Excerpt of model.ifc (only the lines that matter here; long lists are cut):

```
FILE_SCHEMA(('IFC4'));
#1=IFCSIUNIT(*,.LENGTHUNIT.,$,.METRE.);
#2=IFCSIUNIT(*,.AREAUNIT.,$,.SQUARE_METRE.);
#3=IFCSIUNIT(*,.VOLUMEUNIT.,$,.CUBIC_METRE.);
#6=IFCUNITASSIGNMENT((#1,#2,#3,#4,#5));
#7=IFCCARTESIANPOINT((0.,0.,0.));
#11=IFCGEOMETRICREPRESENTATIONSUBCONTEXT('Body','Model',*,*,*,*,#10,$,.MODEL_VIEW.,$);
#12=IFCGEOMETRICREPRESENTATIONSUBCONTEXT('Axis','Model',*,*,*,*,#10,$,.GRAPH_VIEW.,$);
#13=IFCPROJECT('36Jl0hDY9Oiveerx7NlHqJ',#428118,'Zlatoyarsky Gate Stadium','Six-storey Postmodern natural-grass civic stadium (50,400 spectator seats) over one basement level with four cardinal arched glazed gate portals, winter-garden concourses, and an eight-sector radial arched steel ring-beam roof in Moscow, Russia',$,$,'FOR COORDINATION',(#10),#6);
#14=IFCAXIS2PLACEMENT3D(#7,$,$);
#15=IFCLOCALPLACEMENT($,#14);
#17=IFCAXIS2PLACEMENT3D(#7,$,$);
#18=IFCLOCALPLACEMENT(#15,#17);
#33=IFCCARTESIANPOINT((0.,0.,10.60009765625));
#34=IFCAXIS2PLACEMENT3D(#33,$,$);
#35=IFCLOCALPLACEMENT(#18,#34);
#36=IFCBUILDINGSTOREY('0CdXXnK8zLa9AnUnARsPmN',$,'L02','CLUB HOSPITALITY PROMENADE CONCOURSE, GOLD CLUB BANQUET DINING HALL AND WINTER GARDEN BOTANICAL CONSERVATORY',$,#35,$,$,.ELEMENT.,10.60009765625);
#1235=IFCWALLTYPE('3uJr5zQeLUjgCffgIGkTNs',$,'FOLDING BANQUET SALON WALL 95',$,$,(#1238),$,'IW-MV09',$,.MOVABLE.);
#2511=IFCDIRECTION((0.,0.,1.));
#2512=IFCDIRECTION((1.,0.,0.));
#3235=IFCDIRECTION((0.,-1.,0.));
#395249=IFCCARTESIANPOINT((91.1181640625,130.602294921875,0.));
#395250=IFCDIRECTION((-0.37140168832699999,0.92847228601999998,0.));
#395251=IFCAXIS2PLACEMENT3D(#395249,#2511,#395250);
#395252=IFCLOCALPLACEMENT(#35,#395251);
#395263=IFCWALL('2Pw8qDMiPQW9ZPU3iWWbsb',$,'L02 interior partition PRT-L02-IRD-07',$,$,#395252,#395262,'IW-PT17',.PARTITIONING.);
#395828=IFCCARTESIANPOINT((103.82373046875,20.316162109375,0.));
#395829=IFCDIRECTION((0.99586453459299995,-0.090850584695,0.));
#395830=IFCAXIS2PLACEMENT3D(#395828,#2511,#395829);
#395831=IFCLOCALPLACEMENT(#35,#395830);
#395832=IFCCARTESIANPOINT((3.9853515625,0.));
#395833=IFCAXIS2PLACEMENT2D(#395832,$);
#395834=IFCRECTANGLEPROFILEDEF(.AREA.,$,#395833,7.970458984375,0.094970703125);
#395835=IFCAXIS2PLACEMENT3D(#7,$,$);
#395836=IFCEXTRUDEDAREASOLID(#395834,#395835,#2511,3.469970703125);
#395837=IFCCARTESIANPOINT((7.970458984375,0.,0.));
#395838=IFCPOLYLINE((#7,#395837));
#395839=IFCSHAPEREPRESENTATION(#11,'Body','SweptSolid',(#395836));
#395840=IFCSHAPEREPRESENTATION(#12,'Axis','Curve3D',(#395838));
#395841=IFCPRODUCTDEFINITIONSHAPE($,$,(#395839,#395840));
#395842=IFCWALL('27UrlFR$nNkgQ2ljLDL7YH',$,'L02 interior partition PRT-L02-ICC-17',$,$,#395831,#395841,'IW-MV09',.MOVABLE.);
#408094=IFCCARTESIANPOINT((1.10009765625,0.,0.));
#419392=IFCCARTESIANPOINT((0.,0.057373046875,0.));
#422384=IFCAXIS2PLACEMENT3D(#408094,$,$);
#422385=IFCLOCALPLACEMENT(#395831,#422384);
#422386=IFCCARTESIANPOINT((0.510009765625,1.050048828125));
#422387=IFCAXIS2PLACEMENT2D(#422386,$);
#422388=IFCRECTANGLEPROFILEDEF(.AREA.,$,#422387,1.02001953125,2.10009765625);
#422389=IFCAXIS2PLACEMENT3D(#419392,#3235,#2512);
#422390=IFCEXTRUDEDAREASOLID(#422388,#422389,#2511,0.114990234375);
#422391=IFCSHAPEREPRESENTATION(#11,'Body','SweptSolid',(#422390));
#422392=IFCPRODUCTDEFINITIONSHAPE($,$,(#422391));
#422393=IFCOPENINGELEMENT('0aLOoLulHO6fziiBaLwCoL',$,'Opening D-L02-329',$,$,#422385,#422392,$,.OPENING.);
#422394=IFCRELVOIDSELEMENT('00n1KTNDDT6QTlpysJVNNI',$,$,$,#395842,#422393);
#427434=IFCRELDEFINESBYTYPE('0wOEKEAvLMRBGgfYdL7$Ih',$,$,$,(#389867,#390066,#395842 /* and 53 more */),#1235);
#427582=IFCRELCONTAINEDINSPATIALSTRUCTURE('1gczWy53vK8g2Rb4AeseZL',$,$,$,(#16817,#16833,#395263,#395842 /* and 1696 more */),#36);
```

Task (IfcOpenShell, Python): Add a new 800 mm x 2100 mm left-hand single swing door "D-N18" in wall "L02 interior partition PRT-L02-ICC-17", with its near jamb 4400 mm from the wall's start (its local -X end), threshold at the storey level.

```python
import numpy as np
import ifcopenshell
import ifcopenshell.api.feature
import ifcopenshell.api.geometry
import ifcopenshell.api.root
import ifcopenshell.api.spatial
import ifcopenshell.geom
import ifcopenshell.util.element
import ifcopenshell.util.placement
import ifcopenshell.util.representation
import ifcopenshell.util.shape
import ifcopenshell.util.unit

model = ifcopenshell.open("model.ifc")
unit_scale = ifcopenshell.util.unit.calculate_unit_scale(model)
settings = ifcopenshell.geom.settings()


def volume(element):
    """Net volume in cubic metres, openings subtracted."""
    shape = ifcopenshell.geom.create_shape(settings, element)
    return ifcopenshell.util.shape.get_volume(shape.geometry)


wall = model.by_id(395842)
storey = ifcopenshell.util.element.get_container(wall, ifc_class="IfcBuildingStorey")
context = ifcopenshell.util.representation.get_context(model, "Model", "Body", "MODEL_VIEW")
before = volume(wall)

width, height, from_end, sill = 0.8, 2.1, 4.4, 0.0  # metres

# The wall runs along its own X axis, and the end named is its -X end.
wall_shape = ifcopenshell.geom.create_shape(settings, wall)
x, y, z = ifcopenshell.util.shape.get_vertices(wall_shape.geometry).T
start = x.min() + from_end
face, thickness = float(y.min()), float(y.max() - y.min())
wall_matrix = ifcopenshell.util.placement.get_local_placement(wall.ObjectPlacement)
level = ifcopenshell.util.placement.get_local_placement(storey.ObjectPlacement)[2, 3]


def in_wall(x, y):
    """Placement at x, y metres in the wall's axes, at sill height."""
    matrix = wall_matrix.copy()
    matrix[:, 3] = wall_matrix @ np.array([x / unit_scale, y / unit_scale, 0.0, 1.0])
    matrix[2, 3] = level + sill / unit_scale
    return matrix


# Opening: a box that overshoots both wall faces by 50 mm.
opening = ifcopenshell.api.root.create_entity(model, ifc_class="IfcOpeningElement", predefined_type="OPENING")
box = ifcopenshell.api.geometry.add_wall_representation(
    model, context=context, length=width, height=height, thickness=thickness + 0.1
)
ifcopenshell.api.geometry.assign_representation(model, product=opening, representation=box)
ifcopenshell.api.geometry.edit_object_placement(model, product=opening, matrix=in_wall(start, face - 0.05), is_si=False)
ifcopenshell.api.feature.add_feature(model, feature=opening, element=wall)

door = ifcopenshell.api.root.create_entity(model, ifc_class="IfcDoor", name="D-N18", predefined_type="DOOR")
door.OverallWidth, door.OverallHeight = width / unit_scale, height / unit_scale
door.OperationType = "SINGLE_SWING_LEFT"
body = ifcopenshell.api.geometry.add_door_representation(
    model,
    context=context,
    overall_width=door.OverallWidth,
    overall_height=door.OverallHeight,
    operation_type="SINGLE_SWING_LEFT",
    lining_properties={"LiningDepth": thickness / unit_scale, "ThresholdDepth": thickness / unit_scale},
)
ifcopenshell.api.geometry.assign_representation(model, product=door, representation=body)
ifcopenshell.api.spatial.assign_container(model, products=[door], relating_structure=storey)
ifcopenshell.api.feature.add_filling(model, opening=opening, element=door)

# The lining spans the wall, so the door starts at the wall face.
ifcopenshell.api.geometry.edit_object_placement(model, product=door, matrix=in_wall(start, face), is_si=False)

after = volume(wall)

print(f"wall volume {before:.3f} -> {after:.3f} m3")

model.write("model-out.ifc")
```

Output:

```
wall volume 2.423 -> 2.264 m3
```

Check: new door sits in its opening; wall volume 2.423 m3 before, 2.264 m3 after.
